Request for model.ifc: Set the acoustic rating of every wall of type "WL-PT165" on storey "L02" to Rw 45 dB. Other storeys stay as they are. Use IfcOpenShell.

First a look at what the model holds.

```python
import ifcopenshell
import ifcopenshell.util.element

model = ifcopenshell.open("model.ifc")
print(model.schema)
storey = next(s for s in model.by_type("IfcBuildingStorey") if s.Name == "L02")
walls = [e for e in ifcopenshell.util.element.get_decomposition(storey) if e.is_a("IfcWall")]
seen = {}
for e in walls:
    element_type = ifcopenshell.util.element.get_type(e)
    key = (element_type.Name if element_type != e and element_type else None, ifcopenshell.util.element.get_pset(e, "Pset_WallCommon", "AcousticRating"))
    seen[key] = seen.get(key, 0) + 1
for (name, value), count in sorted(seen.items(), key=str):
    print(count, "x", name, "|", value)
```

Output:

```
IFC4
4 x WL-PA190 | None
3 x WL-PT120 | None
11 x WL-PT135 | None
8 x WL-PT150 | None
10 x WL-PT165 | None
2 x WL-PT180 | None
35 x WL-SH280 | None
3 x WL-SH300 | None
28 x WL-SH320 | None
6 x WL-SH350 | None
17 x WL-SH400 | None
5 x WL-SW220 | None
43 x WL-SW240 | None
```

```python
import ifcopenshell
import ifcopenshell.api.pset
import ifcopenshell.util.element

model = ifcopenshell.open("model.ifc")

storey = next(s for s in model.by_type("IfcBuildingStorey") if s.Name == "L02")
walls = [e for e in ifcopenshell.util.element.get_decomposition(storey) if e.is_a("IfcWall")]

count = 0
for e in walls:
    element_type = ifcopenshell.util.element.get_type(e)
    if element_type in (None, e) or element_type.Name != "WL-PT165":
        continue
    # add_pset returns the element's existing set when there is one.
    pset = ifcopenshell.api.pset.add_pset(model, product=e, name="Pset_WallCommon")
    ifcopenshell.api.pset.edit_pset(model, pset=pset, properties={"AcousticRating": "Rw 45 dB"})
    count += 1

print(count, "walls updated")

model.write("model_updated.ifc")
```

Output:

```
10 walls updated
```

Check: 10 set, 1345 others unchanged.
